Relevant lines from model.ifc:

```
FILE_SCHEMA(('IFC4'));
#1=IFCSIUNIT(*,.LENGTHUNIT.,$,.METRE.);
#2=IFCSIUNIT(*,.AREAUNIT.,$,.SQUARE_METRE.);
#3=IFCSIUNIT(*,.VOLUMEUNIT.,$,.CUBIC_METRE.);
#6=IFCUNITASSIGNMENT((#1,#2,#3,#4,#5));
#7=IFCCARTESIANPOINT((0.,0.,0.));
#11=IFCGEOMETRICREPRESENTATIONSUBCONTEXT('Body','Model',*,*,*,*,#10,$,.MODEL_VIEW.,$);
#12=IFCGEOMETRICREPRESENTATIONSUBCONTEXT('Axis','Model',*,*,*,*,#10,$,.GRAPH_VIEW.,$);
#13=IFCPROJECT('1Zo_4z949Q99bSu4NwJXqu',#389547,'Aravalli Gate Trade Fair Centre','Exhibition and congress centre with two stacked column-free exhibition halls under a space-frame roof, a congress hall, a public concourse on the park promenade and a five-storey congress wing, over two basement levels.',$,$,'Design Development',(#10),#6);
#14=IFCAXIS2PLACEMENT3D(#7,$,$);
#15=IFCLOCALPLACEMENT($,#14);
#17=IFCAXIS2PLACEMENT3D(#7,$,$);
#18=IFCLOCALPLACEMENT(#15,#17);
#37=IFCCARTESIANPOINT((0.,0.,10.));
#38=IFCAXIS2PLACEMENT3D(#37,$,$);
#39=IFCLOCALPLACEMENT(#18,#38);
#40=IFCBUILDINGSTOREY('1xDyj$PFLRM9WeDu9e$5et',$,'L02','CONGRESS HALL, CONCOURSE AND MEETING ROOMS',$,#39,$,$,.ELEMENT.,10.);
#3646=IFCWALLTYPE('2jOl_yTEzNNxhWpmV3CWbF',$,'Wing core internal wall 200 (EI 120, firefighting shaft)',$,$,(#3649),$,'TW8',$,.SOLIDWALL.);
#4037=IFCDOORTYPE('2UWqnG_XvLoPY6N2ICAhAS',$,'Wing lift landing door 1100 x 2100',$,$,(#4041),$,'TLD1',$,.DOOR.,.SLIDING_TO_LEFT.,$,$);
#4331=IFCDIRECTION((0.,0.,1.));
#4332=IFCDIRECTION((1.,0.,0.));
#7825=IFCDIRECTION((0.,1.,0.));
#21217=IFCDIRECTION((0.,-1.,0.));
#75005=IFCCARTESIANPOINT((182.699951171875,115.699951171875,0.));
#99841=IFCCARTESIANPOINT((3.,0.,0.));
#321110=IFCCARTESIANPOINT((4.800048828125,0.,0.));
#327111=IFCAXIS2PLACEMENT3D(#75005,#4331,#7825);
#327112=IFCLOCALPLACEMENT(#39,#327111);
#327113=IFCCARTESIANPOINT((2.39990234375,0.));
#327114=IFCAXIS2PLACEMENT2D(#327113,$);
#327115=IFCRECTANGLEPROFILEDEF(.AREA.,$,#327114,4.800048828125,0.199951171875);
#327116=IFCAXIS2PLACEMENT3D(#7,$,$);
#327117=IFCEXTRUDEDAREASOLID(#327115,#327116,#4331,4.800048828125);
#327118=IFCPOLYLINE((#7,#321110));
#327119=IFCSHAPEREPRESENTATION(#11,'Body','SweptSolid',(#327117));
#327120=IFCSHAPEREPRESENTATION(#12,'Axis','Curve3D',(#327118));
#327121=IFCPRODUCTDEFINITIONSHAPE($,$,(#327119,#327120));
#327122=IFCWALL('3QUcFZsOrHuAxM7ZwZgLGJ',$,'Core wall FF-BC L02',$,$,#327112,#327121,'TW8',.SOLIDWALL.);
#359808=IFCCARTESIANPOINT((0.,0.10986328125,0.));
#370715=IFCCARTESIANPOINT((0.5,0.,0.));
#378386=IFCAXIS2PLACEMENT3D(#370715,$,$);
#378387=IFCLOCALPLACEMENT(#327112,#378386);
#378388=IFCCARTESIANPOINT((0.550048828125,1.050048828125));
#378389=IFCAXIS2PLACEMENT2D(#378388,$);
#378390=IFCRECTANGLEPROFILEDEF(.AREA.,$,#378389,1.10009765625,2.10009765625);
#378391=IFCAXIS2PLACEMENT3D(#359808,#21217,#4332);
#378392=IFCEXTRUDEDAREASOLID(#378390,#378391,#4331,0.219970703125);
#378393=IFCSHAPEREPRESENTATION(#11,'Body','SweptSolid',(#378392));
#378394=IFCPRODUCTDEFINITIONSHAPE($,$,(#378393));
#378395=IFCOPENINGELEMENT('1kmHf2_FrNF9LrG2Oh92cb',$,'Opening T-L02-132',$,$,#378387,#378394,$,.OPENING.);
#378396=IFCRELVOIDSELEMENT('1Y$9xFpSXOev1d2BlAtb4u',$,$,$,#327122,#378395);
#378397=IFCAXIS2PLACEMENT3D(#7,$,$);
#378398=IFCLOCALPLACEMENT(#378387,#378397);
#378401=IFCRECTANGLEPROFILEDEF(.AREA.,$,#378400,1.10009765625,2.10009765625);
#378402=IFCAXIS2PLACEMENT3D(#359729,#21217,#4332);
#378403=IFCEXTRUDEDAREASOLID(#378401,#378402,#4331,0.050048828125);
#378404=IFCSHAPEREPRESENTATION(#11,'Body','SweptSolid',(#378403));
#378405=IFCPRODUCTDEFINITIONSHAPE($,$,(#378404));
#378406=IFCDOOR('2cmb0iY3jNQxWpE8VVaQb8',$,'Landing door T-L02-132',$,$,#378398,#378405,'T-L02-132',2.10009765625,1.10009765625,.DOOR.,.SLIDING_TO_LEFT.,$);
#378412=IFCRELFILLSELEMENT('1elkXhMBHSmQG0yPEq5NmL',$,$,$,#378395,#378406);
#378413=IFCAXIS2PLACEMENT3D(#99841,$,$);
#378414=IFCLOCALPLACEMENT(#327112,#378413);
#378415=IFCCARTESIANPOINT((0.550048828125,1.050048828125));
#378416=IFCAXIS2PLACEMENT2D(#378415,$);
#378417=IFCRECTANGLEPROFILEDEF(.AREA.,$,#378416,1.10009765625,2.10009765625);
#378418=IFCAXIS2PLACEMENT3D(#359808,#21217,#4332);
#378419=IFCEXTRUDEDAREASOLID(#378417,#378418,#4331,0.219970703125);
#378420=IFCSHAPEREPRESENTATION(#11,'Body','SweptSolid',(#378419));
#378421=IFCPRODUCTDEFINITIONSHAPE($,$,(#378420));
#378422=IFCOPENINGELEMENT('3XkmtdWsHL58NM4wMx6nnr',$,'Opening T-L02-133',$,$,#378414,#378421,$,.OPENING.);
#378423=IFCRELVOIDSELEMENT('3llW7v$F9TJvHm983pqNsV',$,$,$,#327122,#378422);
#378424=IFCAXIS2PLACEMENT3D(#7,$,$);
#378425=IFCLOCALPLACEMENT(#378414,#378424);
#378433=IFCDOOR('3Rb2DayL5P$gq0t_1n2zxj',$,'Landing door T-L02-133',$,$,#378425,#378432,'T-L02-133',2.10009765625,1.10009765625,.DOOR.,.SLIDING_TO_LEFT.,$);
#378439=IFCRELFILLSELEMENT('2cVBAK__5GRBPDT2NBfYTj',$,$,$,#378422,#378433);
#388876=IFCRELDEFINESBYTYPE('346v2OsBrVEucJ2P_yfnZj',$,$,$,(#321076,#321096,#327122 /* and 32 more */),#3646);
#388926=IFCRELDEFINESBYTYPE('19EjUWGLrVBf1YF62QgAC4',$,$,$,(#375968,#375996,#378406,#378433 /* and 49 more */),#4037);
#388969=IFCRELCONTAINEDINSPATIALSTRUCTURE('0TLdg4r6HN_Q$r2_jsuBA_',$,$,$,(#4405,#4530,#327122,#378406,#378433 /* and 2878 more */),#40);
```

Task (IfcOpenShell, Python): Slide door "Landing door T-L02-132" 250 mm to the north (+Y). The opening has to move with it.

```python
import ifcopenshell
import ifcopenshell.api.geometry
import ifcopenshell.util.placement
import ifcopenshell.util.unit

model = ifcopenshell.open("model.ifc")
unit_scale = ifcopenshell.util.unit.calculate_unit_scale(model)

door = model.by_id(378406)
opening = door.FillsVoids[0].RelatingOpeningElement
wall = opening.VoidsElements[0].RelatingBuildingElement

wall_matrix = ifcopenshell.util.placement.get_local_placement(wall.ObjectPlacement)
shift = wall_matrix[:3, 0] * 0.25 / unit_scale
before = ifcopenshell.util.placement.get_local_placement(door.ObjectPlacement)[:3, 3].copy()

# The door is placed relative to its opening, so it follows when the opening moves.
matrix = ifcopenshell.util.placement.get_local_placement(opening.ObjectPlacement)
matrix[:3, 3] += shift
ifcopenshell.api.geometry.edit_object_placement(
    model, product=opening, matrix=matrix, is_si=False, should_transform_children=True
)

after = ifcopenshell.util.placement.get_local_placement(door.ObjectPlacement)[:3, 3]
print("door moved by", (after - before).round(3) + 0.0)

model.write("model_updated.ifc")
```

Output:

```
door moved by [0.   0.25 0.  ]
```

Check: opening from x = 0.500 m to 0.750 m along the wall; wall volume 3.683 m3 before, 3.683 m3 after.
